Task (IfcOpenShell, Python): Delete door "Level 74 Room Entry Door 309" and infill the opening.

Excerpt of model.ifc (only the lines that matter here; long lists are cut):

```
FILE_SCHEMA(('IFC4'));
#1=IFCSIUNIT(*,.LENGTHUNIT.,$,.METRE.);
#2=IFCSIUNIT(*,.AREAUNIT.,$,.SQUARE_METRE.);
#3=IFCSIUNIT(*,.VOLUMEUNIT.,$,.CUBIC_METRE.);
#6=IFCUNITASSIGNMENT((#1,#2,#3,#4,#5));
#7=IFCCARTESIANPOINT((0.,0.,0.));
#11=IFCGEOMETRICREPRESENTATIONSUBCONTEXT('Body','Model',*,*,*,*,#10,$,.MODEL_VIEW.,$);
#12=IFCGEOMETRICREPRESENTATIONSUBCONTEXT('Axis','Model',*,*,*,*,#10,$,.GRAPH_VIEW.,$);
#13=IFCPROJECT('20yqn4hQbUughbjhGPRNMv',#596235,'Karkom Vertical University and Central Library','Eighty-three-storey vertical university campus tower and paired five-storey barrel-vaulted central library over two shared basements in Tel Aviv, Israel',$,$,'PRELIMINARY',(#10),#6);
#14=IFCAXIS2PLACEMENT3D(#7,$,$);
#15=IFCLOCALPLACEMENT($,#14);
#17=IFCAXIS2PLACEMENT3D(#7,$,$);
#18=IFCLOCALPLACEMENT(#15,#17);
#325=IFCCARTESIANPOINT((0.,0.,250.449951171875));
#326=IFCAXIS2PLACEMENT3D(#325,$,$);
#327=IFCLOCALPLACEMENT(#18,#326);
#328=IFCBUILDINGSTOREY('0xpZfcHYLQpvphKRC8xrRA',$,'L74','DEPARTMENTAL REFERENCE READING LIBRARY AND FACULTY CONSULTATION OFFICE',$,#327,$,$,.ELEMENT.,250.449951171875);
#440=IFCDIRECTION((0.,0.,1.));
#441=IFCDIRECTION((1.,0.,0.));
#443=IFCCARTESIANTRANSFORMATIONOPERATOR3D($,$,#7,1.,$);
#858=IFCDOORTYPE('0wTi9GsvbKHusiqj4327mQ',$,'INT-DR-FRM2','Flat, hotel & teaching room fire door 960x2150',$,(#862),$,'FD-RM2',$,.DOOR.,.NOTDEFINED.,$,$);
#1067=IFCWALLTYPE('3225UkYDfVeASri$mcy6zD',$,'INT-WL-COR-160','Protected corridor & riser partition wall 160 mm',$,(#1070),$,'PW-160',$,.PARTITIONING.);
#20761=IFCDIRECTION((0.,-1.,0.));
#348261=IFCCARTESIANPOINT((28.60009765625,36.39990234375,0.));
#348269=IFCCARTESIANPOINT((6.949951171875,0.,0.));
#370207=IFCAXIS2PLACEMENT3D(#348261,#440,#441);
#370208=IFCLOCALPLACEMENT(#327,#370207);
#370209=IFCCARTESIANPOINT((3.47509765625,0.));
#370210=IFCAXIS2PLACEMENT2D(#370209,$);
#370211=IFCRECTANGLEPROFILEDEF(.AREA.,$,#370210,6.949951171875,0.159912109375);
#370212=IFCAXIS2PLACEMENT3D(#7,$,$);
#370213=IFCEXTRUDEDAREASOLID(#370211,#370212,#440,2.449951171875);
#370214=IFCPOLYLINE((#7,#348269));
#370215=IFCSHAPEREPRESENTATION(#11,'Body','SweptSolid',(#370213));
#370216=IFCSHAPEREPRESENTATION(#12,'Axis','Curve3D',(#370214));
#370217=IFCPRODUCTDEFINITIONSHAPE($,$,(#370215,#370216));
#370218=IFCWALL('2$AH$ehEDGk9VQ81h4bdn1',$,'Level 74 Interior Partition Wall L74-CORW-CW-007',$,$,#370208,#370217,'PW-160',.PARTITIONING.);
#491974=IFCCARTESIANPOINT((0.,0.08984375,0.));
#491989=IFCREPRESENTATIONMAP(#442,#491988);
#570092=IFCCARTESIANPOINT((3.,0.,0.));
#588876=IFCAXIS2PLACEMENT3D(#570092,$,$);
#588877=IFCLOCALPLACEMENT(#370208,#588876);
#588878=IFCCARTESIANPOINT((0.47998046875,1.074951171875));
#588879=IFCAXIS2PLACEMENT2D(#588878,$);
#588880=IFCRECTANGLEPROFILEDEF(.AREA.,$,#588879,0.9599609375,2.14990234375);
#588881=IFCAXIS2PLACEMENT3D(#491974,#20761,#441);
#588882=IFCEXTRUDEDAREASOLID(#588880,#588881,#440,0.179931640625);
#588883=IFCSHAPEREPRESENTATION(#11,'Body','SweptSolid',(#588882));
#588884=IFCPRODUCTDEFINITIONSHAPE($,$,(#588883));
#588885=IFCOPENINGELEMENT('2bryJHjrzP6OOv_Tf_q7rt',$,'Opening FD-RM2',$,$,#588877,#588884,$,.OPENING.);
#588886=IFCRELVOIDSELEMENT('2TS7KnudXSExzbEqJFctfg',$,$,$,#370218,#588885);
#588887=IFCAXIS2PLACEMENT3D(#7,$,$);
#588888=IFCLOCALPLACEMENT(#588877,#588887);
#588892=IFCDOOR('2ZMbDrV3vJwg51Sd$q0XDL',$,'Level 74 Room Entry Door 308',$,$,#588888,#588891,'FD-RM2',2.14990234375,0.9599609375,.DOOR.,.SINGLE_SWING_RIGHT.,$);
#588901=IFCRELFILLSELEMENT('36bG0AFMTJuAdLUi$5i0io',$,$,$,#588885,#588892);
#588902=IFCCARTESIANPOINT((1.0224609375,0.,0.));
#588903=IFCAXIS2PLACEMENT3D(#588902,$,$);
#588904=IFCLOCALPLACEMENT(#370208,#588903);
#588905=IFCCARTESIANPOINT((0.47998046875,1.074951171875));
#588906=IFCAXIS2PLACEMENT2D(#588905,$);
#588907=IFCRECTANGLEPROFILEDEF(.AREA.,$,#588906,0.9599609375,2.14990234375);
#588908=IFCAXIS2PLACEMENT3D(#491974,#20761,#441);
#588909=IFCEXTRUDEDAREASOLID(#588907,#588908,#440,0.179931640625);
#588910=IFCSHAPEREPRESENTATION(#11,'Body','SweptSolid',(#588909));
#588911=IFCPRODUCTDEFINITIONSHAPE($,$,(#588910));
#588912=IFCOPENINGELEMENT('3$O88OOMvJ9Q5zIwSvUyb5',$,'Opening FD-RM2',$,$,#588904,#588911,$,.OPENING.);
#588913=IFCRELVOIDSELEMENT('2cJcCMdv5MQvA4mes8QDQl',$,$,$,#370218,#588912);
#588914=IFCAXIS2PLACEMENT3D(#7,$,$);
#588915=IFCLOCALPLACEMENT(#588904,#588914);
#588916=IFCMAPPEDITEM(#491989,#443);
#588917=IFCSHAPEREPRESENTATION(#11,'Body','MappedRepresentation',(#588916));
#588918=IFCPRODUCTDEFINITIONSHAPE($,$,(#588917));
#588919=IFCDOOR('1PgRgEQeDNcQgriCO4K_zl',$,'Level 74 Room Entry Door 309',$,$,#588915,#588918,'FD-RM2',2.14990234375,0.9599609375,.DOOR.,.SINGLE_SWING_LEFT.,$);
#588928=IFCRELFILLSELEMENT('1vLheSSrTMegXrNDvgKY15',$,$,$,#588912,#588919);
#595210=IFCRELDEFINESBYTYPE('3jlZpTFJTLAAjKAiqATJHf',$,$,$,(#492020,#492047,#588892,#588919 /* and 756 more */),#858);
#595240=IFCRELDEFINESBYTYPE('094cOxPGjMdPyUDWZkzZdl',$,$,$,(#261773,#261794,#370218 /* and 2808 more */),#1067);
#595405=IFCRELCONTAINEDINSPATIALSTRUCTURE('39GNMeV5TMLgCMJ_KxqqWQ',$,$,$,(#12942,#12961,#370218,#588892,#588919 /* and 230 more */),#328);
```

```python
import ifcopenshell
import ifcopenshell.api.feature
import ifcopenshell.api.root
import ifcopenshell.geom
import ifcopenshell.util.shape

model = ifcopenshell.open("model.ifc")
settings = ifcopenshell.geom.settings()


def volume(element):
    """Net volume in cubic metres, openings subtracted."""
    shape = ifcopenshell.geom.create_shape(settings, element)
    return ifcopenshell.util.shape.get_volume(shape.geometry)


door = model.by_guid("1PgRgEQeDNcQgriCO4K_zl")
opening = door.FillsVoids[0].RelatingOpeningElement
wall = opening.VoidsElements[0].RelatingBuildingElement
before = volume(wall)

ifcopenshell.api.root.remove_product(model, product=door)
ifcopenshell.api.feature.remove_feature(model, feature=opening)

after = volume(wall)

print(f"wall volume {before:.3f} -> {after:.3f} m3")

model.write("model_updated.ifc")
```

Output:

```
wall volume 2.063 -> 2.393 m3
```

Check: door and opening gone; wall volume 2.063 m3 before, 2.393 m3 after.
